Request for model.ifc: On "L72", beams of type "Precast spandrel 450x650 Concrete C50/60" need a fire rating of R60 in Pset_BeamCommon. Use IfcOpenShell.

First a look at what the model holds.

```python
import ifcopenshell
import ifcopenshell.util.element

model = ifcopenshell.open("model.ifc")
print(model.schema)
storey = next(s for s in model.by_type("IfcBuildingStorey") if s.Name == "L72")
beams = [e for e in ifcopenshell.util.element.get_decomposition(storey) if e.is_a("IfcBeam")]
seen = {}
for e in beams:
    element_type = ifcopenshell.util.element.get_type(e)
    key = (element_type.Name if element_type != e and element_type else None, ifcopenshell.util.element.get_pset(e, "Pset_BeamCommon", "FireRating"))
    seen[key] = seen.get(key, 0) + 1
for (name, value), count in sorted(seen.items(), key=str):
    print(count, "x", name, "|", value)
```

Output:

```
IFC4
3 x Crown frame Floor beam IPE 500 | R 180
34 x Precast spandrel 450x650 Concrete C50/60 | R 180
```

```python
import ifcopenshell
import ifcopenshell.api.pset
import ifcopenshell.util.element

model = ifcopenshell.open("model.ifc")

storey = next(s for s in model.by_type("IfcBuildingStorey") if s.Name == "L72")
beams = [e for e in ifcopenshell.util.element.get_decomposition(storey) if e.is_a("IfcBeam")]

count = 0
for e in beams:
    element_type = ifcopenshell.util.element.get_type(e)
    if element_type in (None, e) or element_type.Name != "Precast spandrel 450x650 Concrete C50/60":
        continue
    found = ifcopenshell.util.element.get_pset(e, "Pset_BeamCommon", should_inherit=False)
    if found:
        pset = model.by_id(found["id"])
        if len(ifcopenshell.util.element.get_elements_by_pset(pset)) > 1:
            pset = ifcopenshell.api.pset.unshare_pset(model, products=[e], pset=pset)[0]
    else:
        pset = ifcopenshell.api.pset.add_pset(model, product=e, name="Pset_BeamCommon")
    ifcopenshell.api.pset.edit_pset(model, pset=pset, properties={"FireRating": "R60"})
    count += 1

print(count, "beams updated")

model.write("model_v2.ifc")
```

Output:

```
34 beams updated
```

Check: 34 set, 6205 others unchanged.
